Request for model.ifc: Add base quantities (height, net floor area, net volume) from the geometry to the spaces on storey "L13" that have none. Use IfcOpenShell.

First a look at what the model holds.

```python
import ifcopenshell
import ifcopenshell.util.element
import ifcopenshell.util.unit

model = ifcopenshell.open("model.ifc")
print(model.schema)
for unit_type in ("LENGTHUNIT", "AREAUNIT", "VOLUMEUNIT"):
    print(unit_type, ifcopenshell.util.unit.calculate_unit_scale(model, unit_type))
storey = next(s for s in model.by_type("IfcBuildingStorey") if s.Name == "L13")
spaces = [e for e in ifcopenshell.util.element.get_decomposition(storey) if e.is_a("IfcSpace")]
for e in sorted(spaces, key=lambda e: e.id()):
    print(e.id(), e.is_a(), e.Name, list(ifcopenshell.util.element.get_psets(e, qtos_only=True)), sep=" | ")
```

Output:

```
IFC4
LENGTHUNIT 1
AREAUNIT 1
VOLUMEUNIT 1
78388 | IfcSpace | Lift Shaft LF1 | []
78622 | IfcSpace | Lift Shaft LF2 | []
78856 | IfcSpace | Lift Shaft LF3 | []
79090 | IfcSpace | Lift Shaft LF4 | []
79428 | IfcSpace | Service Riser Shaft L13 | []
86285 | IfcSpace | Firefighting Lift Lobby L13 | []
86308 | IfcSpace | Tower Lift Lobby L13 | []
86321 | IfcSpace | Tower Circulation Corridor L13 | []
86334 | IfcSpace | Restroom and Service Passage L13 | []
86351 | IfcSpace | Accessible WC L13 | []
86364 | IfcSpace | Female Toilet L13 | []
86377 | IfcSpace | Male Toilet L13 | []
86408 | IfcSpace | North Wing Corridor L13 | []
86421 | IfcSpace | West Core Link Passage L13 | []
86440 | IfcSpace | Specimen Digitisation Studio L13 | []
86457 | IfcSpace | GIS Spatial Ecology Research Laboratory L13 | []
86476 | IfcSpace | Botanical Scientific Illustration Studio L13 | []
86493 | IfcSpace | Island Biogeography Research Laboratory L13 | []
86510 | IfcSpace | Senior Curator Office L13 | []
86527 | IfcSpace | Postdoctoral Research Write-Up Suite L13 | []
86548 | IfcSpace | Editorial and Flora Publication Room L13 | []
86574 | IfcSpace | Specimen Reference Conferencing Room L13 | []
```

```python
import ifcopenshell
import ifcopenshell.api.pset
import ifcopenshell.geom
import ifcopenshell.util.element
import ifcopenshell.util.shape
import ifcopenshell.util.unit

model = ifcopenshell.open("model.ifc")
unit_scale = ifcopenshell.util.unit.calculate_unit_scale(model)
area_scale = ifcopenshell.util.unit.calculate_unit_scale(model, "AREAUNIT")
volume_scale = ifcopenshell.util.unit.calculate_unit_scale(model, "VOLUMEUNIT")
settings = ifcopenshell.geom.settings()

storey = next(s for s in model.by_type("IfcBuildingStorey") if s.Name == "L13")
spaces = [e for e in ifcopenshell.util.element.get_decomposition(storey) if e.is_a("IfcSpace")]

for e in sorted(spaces, key=lambda e: e.id()):
    if ifcopenshell.util.element.get_psets(e, qtos_only=True, should_inherit=False):
        continue
    # Geometry comes back in metres, in the element's own axes.
    shape = ifcopenshell.geom.create_shape(settings, e)
    values = {
        "Height": ifcopenshell.util.shape.get_z(shape.geometry) / unit_scale,
        "NetFloorArea": ifcopenshell.util.shape.get_footprint_area(shape.geometry) / area_scale,
        "NetVolume": ifcopenshell.util.shape.get_volume(shape.geometry) / volume_scale,
    }
    qto = ifcopenshell.api.pset.add_qto(model, product=e, name="Qto_SpaceBaseQuantities")
    ifcopenshell.api.pset.edit_qto(model, qto=qto, properties=values)
    print(e.id(), {k: round(v, 3) for k, v in values.items()})

model.write("model-out.ifc")
```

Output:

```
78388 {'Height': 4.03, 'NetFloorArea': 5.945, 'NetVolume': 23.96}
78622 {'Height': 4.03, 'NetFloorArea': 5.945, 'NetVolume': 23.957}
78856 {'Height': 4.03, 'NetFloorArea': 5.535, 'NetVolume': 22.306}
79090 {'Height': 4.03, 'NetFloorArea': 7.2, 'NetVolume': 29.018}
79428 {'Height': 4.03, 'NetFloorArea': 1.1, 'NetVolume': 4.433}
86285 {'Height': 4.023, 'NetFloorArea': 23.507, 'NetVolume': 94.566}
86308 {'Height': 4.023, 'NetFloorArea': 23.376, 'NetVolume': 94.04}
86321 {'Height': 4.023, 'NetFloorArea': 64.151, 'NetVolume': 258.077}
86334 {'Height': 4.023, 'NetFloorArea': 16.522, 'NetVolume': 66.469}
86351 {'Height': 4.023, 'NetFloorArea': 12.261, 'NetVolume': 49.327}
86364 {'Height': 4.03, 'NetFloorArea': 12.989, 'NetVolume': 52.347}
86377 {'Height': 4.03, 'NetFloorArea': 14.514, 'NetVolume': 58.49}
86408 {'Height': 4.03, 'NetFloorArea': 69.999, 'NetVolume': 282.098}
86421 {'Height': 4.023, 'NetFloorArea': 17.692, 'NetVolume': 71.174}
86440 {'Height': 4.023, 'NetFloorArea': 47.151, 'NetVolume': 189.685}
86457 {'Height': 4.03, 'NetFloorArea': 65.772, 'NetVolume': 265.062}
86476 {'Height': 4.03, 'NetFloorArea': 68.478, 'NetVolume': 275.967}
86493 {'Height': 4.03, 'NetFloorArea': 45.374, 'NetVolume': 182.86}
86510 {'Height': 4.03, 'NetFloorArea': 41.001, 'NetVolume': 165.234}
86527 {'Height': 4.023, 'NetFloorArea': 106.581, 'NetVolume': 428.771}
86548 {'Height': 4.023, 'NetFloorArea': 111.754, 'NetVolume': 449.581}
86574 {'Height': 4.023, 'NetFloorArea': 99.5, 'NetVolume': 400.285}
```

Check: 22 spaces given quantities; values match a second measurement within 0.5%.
